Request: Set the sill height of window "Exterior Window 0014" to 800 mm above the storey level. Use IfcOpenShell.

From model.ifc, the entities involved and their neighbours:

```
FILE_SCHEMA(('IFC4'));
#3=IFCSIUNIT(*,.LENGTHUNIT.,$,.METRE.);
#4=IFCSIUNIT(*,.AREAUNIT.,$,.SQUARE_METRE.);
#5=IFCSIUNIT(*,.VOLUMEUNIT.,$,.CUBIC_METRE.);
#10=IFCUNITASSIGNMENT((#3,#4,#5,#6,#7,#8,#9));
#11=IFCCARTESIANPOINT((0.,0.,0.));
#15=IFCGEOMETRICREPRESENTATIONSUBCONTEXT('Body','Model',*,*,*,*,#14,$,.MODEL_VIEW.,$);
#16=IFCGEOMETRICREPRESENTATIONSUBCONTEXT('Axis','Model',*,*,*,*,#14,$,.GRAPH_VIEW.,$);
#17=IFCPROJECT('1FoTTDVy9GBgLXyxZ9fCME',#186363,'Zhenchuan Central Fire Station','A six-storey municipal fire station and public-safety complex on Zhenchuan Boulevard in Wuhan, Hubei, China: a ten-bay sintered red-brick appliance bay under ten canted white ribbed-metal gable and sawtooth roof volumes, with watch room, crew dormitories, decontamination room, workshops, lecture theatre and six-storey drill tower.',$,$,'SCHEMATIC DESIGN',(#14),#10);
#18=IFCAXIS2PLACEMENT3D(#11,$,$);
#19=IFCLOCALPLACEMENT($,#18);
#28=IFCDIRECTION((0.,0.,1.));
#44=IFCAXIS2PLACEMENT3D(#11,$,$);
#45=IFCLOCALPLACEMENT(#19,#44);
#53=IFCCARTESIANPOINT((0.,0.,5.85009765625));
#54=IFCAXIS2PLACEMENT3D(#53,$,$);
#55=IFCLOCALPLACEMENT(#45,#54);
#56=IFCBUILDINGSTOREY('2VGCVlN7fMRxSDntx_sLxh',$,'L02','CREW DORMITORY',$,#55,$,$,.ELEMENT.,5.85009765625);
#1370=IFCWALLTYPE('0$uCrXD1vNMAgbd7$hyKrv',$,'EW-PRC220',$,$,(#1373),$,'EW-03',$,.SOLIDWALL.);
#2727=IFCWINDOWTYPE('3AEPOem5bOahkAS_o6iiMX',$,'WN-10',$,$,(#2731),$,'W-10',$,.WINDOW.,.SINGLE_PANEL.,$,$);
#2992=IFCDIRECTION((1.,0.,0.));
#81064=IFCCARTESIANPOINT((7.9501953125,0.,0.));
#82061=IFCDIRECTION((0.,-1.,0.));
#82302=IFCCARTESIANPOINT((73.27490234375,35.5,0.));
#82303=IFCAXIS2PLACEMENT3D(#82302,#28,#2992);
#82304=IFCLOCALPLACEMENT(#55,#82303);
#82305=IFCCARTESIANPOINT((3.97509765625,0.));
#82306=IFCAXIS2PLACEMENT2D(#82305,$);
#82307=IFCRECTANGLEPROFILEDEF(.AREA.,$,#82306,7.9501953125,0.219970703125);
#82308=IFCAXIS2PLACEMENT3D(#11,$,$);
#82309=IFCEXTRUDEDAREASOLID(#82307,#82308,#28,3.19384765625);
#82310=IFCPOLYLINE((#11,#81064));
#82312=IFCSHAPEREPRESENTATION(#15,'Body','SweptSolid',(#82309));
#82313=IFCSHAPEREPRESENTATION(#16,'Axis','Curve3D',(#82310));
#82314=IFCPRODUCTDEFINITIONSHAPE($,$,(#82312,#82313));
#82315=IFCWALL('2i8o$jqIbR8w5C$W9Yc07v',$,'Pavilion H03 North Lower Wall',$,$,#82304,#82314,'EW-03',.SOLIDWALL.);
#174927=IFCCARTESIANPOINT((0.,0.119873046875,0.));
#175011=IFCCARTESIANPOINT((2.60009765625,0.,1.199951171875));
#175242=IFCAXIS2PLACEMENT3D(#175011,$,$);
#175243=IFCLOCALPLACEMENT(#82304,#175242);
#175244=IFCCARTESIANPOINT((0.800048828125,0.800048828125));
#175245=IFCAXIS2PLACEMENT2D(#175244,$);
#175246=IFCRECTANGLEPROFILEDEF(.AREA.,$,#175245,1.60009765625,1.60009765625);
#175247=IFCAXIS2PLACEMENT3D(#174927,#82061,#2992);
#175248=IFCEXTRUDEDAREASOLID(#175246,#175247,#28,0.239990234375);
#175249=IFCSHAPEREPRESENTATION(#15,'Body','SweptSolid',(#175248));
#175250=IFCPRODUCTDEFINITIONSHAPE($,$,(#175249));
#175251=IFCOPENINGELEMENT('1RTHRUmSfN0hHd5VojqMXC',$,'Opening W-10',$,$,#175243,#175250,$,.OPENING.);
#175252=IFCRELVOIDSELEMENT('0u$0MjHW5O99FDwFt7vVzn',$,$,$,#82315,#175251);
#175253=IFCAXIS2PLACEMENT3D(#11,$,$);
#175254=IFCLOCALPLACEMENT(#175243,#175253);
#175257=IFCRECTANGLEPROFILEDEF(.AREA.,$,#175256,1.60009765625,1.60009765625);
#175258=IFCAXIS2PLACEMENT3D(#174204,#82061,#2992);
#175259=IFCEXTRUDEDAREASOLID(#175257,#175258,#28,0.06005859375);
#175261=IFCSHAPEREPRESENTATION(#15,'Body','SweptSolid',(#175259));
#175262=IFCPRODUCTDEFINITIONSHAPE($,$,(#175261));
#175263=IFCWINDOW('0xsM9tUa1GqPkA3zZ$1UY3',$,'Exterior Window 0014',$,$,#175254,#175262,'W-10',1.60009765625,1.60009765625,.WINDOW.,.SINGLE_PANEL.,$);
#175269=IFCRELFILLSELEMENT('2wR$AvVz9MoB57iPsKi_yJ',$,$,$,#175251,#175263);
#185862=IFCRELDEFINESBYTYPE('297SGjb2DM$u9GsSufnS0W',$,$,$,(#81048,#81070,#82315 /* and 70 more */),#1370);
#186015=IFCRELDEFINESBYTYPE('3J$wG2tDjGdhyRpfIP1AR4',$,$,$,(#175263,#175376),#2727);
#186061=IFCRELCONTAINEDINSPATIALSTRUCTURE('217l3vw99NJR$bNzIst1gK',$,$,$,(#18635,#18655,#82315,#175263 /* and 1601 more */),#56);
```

```python
import numpy as np
import ifcopenshell
import ifcopenshell.api.geometry
import ifcopenshell.geom
import ifcopenshell.util.element
import ifcopenshell.util.placement
import ifcopenshell.util.shape
import ifcopenshell.util.unit

model = ifcopenshell.open("model.ifc")
unit_scale = ifcopenshell.util.unit.calculate_unit_scale(model)

window = model.by_id(175263)
opening = window.FillsVoids[0].RelatingOpeningElement
storey = ifcopenshell.util.element.get_container(window, ifc_class="IfcBuildingStorey")
level = ifcopenshell.util.placement.get_local_placement(storey.ObjectPlacement)[2, 3]

# The opening's origin need not be at the sill, so measure its lowest point.
shape = ifcopenshell.geom.create_shape(ifcopenshell.geom.settings(), opening)
bottom = ifcopenshell.util.shape.get_shape_bottom_elevation(shape, shape.geometry) / unit_scale
dz = level + 0.8 / unit_scale - bottom

shift = np.array([0.0, 0.0, dz])
# The window is placed relative to its opening, so it follows when the opening moves.
matrix = ifcopenshell.util.placement.get_local_placement(opening.ObjectPlacement)
matrix[:3, 3] += shift
ifcopenshell.api.geometry.edit_object_placement(
    model, product=opening, matrix=matrix, is_si=False, should_transform_children=True
)

print(f"moved by {dz * unit_scale:+.3f} m")

model.write("model_rev.ifc")
```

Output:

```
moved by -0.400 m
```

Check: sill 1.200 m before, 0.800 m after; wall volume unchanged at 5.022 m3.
